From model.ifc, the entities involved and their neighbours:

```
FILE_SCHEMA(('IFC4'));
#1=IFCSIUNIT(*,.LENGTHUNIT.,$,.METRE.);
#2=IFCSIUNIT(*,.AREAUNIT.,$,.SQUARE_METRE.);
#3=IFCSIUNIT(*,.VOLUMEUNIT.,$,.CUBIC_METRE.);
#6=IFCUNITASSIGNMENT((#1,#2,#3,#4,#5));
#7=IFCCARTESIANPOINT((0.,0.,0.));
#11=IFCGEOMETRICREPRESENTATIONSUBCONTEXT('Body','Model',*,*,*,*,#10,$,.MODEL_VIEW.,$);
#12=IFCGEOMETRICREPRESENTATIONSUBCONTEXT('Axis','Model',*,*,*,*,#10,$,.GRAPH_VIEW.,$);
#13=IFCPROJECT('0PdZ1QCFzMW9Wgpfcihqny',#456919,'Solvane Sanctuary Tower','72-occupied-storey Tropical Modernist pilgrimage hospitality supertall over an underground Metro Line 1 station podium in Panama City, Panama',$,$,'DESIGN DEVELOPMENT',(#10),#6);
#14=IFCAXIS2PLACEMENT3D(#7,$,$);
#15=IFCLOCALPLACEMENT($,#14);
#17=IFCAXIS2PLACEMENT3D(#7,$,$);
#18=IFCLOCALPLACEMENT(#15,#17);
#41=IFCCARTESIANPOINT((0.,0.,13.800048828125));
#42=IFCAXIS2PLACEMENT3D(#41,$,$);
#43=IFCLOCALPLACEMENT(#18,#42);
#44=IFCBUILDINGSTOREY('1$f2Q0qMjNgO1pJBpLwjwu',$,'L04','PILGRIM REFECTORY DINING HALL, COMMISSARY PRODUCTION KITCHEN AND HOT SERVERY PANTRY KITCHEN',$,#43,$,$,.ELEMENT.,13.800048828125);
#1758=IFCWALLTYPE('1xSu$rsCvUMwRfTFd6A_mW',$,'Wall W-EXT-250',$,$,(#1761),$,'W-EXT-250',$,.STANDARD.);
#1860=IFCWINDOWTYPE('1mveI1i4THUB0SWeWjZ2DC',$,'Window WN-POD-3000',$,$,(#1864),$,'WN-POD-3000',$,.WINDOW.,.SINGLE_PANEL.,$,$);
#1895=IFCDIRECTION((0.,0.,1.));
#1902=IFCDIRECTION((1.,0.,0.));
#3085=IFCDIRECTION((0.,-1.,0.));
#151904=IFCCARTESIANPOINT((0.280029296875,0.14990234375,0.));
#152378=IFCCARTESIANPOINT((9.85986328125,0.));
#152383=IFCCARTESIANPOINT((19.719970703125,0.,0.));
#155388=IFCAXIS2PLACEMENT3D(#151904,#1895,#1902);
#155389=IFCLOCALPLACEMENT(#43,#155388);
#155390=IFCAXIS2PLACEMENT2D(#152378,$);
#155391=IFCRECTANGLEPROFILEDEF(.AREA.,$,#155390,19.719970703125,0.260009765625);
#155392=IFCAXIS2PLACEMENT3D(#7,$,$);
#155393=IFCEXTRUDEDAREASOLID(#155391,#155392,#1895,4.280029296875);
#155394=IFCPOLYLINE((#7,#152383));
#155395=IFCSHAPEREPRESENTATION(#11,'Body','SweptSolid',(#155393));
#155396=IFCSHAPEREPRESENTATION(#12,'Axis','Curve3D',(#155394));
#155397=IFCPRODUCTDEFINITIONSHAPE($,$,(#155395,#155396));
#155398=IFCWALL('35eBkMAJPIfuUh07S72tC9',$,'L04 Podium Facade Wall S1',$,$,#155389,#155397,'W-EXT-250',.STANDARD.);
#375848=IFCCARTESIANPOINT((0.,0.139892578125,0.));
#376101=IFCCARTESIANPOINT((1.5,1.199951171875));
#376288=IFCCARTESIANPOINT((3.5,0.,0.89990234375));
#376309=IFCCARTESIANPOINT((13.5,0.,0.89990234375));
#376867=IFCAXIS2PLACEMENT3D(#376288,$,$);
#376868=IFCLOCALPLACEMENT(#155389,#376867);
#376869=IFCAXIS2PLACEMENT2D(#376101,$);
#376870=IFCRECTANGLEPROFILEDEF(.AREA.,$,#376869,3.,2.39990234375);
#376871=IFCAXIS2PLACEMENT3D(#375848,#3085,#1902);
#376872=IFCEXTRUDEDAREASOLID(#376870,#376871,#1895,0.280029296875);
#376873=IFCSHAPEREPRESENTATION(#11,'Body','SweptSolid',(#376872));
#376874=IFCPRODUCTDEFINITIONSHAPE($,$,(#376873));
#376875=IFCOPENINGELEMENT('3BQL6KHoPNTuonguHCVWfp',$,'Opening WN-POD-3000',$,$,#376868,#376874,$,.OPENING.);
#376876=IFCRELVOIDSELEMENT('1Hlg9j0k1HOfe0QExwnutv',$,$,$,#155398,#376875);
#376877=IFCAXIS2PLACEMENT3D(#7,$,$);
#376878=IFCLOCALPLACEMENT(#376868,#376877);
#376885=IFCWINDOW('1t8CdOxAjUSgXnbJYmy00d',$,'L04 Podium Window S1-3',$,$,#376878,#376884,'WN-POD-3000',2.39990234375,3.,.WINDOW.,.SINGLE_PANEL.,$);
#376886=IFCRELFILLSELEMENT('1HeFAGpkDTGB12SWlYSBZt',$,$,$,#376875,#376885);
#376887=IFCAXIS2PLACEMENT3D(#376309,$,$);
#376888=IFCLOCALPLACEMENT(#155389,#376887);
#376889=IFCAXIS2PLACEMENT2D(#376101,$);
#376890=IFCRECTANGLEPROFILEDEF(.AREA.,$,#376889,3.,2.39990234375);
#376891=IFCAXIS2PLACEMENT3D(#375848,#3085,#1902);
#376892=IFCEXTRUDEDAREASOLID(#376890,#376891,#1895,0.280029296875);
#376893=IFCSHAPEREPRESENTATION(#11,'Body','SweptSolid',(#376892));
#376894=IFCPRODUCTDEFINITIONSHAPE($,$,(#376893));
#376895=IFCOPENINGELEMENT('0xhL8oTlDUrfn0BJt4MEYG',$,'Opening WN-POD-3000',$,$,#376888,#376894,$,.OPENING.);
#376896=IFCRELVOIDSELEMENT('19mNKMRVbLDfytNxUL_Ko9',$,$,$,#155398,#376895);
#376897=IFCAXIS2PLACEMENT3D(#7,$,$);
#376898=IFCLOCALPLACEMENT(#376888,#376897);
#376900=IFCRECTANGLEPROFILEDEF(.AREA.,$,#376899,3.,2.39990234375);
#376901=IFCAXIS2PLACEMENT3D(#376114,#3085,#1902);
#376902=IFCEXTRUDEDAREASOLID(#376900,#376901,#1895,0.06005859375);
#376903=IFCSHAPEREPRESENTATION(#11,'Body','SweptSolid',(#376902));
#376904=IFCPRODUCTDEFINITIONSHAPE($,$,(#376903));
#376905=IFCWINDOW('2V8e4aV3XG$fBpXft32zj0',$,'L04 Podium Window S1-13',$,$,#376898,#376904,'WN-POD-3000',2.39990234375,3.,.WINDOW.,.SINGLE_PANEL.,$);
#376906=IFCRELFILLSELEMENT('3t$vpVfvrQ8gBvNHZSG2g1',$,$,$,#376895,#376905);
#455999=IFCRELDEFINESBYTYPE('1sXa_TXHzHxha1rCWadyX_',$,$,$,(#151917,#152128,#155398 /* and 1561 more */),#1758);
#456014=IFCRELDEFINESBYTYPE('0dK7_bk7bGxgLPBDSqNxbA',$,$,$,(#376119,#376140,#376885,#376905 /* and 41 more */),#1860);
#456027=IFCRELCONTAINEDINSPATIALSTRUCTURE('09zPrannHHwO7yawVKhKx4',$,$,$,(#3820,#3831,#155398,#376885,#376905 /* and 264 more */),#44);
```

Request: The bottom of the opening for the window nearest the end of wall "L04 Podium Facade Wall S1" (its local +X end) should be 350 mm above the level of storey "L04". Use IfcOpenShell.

```python
import numpy as np
import ifcopenshell
import ifcopenshell.api.geometry
import ifcopenshell.geom
import ifcopenshell.util.element
import ifcopenshell.util.placement
import ifcopenshell.util.shape
import ifcopenshell.util.unit

model = ifcopenshell.open("model.ifc")
unit_scale = ifcopenshell.util.unit.calculate_unit_scale(model)

window = model.by_id(376905)
opening = window.FillsVoids[0].RelatingOpeningElement
storey = ifcopenshell.util.element.get_container(window, ifc_class="IfcBuildingStorey")
level = ifcopenshell.util.placement.get_local_placement(storey.ObjectPlacement)[2, 3]

# The opening's origin need not be at the sill, so measure its lowest point.
shape = ifcopenshell.geom.create_shape(ifcopenshell.geom.settings(), opening)
bottom = ifcopenshell.util.shape.get_shape_bottom_elevation(shape, shape.geometry) / unit_scale
dz = level + 0.35 / unit_scale - bottom

shift = np.array([0.0, 0.0, dz])
# The window is placed relative to its opening, so it follows when the opening moves.
matrix = ifcopenshell.util.placement.get_local_placement(opening.ObjectPlacement)
matrix[:3, 3] += shift
ifcopenshell.api.geometry.edit_object_placement(
    model, product=opening, matrix=matrix, is_si=False, should_transform_children=True
)

print(f"moved by {dz * unit_scale:+.3f} m")

model.write("model_rev.ifc")
```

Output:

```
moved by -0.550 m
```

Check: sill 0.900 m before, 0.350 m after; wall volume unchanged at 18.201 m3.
